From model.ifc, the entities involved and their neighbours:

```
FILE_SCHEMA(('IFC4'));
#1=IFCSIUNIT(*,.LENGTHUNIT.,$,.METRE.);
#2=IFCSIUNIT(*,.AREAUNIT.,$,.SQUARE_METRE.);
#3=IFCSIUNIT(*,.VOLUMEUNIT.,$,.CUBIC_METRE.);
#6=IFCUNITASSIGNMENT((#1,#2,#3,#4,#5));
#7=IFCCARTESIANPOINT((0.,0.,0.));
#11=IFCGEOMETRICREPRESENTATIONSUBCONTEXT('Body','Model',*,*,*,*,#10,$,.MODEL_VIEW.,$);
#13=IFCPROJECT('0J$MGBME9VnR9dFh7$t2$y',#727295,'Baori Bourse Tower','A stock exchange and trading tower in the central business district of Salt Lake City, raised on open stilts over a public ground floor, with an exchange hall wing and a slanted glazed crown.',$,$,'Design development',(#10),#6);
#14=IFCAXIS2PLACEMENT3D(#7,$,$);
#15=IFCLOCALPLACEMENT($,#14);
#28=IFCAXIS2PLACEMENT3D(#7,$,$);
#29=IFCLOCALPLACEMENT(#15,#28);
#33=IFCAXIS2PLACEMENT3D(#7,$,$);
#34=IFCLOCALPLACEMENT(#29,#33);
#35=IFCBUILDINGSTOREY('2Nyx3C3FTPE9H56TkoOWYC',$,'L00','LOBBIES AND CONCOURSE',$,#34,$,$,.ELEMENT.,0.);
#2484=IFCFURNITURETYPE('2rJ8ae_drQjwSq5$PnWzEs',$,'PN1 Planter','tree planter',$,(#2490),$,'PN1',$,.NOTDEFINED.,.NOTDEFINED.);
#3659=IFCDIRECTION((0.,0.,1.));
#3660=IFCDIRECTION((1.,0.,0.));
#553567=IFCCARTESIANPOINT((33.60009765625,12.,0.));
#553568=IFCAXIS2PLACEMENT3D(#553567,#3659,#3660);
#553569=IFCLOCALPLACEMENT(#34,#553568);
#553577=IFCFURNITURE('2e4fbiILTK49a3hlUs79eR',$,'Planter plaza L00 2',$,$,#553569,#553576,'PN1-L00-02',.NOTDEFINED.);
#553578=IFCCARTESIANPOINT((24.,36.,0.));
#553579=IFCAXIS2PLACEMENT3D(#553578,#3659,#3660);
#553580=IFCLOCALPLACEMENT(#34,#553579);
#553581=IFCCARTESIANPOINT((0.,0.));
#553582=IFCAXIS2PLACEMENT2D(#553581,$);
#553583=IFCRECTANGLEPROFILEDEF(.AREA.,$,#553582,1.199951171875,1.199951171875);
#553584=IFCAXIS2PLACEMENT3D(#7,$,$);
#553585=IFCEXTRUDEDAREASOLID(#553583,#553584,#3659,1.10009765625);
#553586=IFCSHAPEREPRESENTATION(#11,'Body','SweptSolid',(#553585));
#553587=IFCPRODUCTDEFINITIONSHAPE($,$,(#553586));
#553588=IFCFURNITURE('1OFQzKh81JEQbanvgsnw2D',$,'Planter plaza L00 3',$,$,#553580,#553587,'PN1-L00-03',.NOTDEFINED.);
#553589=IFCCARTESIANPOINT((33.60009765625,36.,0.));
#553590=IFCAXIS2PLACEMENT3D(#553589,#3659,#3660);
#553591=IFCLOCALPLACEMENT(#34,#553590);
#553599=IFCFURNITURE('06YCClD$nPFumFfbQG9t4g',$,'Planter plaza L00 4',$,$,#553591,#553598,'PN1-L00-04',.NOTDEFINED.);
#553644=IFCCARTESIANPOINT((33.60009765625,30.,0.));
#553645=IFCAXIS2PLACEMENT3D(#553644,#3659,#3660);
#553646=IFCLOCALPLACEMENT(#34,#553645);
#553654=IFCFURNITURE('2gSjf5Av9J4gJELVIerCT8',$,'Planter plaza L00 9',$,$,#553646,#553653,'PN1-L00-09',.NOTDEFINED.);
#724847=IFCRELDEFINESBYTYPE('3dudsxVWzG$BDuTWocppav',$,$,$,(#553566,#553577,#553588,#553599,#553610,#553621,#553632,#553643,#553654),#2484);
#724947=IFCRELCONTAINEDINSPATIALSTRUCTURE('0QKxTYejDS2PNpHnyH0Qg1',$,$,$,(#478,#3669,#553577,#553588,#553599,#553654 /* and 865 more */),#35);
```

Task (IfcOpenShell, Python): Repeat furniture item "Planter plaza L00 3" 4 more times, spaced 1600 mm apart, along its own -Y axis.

```python
import ifcopenshell
import ifcopenshell.api.geometry
import ifcopenshell.api.root
import ifcopenshell.util.element
import ifcopenshell.util.placement
import ifcopenshell.util.unit

model = ifcopenshell.open("model.ifc")
unit_scale = ifcopenshell.util.unit.calculate_unit_scale(model)

source = model.by_guid("1OFQzKh81JEQbanvgsnw2D")
base = ifcopenshell.util.placement.get_local_placement(source.ObjectPlacement)
step = -base[:3, 1] * 1.6 / unit_scale

for i in range(1, 5):
    copy = ifcopenshell.api.root.copy_class(model, product=source)
    copy.Representation = ifcopenshell.util.element.copy_deep(
        model, source.Representation, exclude=["IfcGeometricRepresentationContext", "IfcRepresentationMap"]
    )
    copy.Tag = None
    matrix = base.copy()
    matrix[:3, 3] += i * step
    print("added at", matrix[:3, 3].round(3) + 0.0)
    ifcopenshell.api.geometry.edit_object_placement(model, product=copy, matrix=matrix, is_si=False)

model.write("model_updated.ifc")
```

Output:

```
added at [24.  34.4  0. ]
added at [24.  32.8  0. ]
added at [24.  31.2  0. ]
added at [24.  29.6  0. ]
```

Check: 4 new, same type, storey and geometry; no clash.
